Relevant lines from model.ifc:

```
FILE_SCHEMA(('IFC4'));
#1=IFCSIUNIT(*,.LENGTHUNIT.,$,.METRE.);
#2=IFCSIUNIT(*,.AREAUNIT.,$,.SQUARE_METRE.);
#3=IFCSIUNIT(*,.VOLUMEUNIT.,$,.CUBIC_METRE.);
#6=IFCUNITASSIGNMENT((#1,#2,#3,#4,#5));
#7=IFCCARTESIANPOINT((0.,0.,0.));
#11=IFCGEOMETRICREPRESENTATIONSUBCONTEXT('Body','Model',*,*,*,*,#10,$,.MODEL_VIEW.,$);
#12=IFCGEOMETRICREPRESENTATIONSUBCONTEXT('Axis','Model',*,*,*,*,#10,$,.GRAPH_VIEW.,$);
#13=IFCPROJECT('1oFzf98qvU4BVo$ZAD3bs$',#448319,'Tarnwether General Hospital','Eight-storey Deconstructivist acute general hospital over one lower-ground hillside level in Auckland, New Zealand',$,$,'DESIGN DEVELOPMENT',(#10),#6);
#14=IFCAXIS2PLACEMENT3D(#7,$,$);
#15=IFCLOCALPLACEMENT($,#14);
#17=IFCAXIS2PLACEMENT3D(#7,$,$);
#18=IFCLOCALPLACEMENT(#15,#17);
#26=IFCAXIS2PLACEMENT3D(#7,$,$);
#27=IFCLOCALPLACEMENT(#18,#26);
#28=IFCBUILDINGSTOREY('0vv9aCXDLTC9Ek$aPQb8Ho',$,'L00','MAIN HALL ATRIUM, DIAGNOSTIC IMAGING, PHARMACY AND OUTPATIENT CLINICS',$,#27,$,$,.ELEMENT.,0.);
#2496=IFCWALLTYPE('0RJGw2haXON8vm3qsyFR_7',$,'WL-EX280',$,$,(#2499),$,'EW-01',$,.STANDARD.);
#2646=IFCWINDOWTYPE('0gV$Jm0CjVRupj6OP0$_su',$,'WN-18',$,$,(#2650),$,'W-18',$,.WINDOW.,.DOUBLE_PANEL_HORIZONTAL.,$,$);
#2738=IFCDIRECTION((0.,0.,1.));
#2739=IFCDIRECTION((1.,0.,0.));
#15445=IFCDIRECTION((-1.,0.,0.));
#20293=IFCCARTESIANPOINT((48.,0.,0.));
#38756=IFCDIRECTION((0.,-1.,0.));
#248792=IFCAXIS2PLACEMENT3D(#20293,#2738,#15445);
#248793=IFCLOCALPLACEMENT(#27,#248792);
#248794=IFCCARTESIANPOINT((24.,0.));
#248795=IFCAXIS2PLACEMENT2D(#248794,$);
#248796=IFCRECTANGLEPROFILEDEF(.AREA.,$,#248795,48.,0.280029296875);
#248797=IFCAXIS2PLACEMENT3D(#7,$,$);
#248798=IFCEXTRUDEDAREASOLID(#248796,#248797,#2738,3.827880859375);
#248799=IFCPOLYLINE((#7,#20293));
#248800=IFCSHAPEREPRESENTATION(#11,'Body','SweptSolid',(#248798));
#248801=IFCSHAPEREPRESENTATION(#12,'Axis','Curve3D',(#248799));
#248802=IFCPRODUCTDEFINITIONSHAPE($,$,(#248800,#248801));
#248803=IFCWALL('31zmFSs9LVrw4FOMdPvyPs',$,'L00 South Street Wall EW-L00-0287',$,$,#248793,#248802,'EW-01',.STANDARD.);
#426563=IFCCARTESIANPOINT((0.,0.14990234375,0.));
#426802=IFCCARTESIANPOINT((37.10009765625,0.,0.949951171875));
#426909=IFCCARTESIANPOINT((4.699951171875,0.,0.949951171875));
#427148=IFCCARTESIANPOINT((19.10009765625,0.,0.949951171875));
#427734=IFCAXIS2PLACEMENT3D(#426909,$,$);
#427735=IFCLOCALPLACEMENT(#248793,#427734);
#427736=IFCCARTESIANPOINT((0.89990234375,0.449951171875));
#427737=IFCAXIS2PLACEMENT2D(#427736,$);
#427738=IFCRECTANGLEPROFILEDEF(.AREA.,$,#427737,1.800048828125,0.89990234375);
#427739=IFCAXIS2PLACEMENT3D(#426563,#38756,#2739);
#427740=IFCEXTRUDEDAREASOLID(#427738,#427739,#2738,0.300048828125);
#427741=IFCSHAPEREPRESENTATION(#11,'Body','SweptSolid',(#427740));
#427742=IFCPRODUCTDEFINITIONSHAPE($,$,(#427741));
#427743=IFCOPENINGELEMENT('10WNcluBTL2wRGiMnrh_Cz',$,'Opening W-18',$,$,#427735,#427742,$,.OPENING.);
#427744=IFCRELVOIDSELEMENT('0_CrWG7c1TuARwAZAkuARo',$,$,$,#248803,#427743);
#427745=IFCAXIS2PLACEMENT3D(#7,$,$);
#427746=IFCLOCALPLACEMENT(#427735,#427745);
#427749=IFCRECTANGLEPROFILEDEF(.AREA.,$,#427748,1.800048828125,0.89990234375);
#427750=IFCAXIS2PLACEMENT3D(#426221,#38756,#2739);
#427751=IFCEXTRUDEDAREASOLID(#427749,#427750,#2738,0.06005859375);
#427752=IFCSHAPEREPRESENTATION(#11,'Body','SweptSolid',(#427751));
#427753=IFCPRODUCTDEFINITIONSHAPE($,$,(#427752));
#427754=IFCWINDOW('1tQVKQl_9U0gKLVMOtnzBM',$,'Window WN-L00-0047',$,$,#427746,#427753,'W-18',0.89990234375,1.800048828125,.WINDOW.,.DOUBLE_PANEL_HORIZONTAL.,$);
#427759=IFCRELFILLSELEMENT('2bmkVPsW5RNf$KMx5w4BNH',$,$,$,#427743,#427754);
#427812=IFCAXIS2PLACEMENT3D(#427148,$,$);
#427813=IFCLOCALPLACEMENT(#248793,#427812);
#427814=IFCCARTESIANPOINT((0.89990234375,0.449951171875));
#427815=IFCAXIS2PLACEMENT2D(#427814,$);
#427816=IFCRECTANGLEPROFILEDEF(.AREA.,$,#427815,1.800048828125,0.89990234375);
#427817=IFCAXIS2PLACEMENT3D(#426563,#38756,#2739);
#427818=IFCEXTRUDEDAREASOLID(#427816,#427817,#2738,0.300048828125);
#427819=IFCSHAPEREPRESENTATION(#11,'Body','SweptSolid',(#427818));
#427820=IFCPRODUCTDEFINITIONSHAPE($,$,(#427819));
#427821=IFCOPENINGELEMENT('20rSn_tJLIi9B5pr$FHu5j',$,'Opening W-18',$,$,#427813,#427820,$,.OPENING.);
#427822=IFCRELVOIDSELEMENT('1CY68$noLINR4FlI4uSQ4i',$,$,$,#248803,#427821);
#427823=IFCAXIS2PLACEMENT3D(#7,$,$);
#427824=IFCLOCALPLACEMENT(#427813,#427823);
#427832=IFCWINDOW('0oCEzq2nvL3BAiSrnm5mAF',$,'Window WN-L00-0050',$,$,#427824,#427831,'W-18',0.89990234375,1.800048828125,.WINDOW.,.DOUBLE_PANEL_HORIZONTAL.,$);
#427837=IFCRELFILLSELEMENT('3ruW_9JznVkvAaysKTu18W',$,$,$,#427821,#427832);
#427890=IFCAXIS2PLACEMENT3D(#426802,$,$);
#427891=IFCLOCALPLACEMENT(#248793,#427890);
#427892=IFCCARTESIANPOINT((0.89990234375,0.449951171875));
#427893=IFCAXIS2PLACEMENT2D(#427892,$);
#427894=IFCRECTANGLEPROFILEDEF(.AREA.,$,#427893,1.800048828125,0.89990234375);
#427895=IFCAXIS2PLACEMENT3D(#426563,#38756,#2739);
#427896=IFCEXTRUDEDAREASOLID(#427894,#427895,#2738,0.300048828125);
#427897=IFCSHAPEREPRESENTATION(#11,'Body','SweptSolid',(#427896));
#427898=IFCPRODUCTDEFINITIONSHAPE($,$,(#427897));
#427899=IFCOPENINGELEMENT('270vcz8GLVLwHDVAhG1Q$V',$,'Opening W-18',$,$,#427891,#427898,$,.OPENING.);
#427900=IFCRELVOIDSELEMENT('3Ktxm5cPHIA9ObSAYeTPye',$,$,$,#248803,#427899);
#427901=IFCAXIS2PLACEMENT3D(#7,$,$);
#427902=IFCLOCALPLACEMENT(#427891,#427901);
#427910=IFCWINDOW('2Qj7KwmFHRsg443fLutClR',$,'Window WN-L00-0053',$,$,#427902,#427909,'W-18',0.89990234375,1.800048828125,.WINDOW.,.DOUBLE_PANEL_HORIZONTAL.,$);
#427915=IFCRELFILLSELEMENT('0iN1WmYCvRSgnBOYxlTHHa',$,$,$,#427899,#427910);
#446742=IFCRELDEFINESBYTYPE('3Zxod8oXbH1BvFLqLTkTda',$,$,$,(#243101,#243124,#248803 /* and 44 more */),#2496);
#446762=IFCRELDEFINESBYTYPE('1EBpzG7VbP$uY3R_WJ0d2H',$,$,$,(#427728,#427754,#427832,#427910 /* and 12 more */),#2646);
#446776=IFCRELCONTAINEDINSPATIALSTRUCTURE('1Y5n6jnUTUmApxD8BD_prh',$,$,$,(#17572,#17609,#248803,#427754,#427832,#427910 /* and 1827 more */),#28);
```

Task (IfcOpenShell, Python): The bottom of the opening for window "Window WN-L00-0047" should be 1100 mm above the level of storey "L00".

```python
import numpy as np
import ifcopenshell
import ifcopenshell.api.geometry
import ifcopenshell.geom
import ifcopenshell.util.element
import ifcopenshell.util.placement
import ifcopenshell.util.shape
import ifcopenshell.util.unit

model = ifcopenshell.open("model.ifc")
unit_scale = ifcopenshell.util.unit.calculate_unit_scale(model)

window = model.by_id(427754)
opening = window.FillsVoids[0].RelatingOpeningElement
storey = ifcopenshell.util.element.get_container(window, ifc_class="IfcBuildingStorey")
level = ifcopenshell.util.placement.get_local_placement(storey.ObjectPlacement)[2, 3]

# The opening's origin need not be at the sill, so measure its lowest point.
shape = ifcopenshell.geom.create_shape(ifcopenshell.geom.settings(), opening)
bottom = ifcopenshell.util.shape.get_shape_bottom_elevation(shape, shape.geometry) / unit_scale
dz = level + 1.1 - bottom

shift = np.array([0.0, 0.0, dz])
# The window is placed relative to its opening, so it follows when the opening moves.
matrix = ifcopenshell.util.placement.get_local_placement(opening.ObjectPlacement)
matrix[:3, 3] += shift
ifcopenshell.api.geometry.edit_object_placement(
    model, product=opening, matrix=matrix, is_si=False, should_transform_children=True
)

print(f"moved by {dz * unit_scale:+.3f} m")

model.write("model_v2.ifc")
```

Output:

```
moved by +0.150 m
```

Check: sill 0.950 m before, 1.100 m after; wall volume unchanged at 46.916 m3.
